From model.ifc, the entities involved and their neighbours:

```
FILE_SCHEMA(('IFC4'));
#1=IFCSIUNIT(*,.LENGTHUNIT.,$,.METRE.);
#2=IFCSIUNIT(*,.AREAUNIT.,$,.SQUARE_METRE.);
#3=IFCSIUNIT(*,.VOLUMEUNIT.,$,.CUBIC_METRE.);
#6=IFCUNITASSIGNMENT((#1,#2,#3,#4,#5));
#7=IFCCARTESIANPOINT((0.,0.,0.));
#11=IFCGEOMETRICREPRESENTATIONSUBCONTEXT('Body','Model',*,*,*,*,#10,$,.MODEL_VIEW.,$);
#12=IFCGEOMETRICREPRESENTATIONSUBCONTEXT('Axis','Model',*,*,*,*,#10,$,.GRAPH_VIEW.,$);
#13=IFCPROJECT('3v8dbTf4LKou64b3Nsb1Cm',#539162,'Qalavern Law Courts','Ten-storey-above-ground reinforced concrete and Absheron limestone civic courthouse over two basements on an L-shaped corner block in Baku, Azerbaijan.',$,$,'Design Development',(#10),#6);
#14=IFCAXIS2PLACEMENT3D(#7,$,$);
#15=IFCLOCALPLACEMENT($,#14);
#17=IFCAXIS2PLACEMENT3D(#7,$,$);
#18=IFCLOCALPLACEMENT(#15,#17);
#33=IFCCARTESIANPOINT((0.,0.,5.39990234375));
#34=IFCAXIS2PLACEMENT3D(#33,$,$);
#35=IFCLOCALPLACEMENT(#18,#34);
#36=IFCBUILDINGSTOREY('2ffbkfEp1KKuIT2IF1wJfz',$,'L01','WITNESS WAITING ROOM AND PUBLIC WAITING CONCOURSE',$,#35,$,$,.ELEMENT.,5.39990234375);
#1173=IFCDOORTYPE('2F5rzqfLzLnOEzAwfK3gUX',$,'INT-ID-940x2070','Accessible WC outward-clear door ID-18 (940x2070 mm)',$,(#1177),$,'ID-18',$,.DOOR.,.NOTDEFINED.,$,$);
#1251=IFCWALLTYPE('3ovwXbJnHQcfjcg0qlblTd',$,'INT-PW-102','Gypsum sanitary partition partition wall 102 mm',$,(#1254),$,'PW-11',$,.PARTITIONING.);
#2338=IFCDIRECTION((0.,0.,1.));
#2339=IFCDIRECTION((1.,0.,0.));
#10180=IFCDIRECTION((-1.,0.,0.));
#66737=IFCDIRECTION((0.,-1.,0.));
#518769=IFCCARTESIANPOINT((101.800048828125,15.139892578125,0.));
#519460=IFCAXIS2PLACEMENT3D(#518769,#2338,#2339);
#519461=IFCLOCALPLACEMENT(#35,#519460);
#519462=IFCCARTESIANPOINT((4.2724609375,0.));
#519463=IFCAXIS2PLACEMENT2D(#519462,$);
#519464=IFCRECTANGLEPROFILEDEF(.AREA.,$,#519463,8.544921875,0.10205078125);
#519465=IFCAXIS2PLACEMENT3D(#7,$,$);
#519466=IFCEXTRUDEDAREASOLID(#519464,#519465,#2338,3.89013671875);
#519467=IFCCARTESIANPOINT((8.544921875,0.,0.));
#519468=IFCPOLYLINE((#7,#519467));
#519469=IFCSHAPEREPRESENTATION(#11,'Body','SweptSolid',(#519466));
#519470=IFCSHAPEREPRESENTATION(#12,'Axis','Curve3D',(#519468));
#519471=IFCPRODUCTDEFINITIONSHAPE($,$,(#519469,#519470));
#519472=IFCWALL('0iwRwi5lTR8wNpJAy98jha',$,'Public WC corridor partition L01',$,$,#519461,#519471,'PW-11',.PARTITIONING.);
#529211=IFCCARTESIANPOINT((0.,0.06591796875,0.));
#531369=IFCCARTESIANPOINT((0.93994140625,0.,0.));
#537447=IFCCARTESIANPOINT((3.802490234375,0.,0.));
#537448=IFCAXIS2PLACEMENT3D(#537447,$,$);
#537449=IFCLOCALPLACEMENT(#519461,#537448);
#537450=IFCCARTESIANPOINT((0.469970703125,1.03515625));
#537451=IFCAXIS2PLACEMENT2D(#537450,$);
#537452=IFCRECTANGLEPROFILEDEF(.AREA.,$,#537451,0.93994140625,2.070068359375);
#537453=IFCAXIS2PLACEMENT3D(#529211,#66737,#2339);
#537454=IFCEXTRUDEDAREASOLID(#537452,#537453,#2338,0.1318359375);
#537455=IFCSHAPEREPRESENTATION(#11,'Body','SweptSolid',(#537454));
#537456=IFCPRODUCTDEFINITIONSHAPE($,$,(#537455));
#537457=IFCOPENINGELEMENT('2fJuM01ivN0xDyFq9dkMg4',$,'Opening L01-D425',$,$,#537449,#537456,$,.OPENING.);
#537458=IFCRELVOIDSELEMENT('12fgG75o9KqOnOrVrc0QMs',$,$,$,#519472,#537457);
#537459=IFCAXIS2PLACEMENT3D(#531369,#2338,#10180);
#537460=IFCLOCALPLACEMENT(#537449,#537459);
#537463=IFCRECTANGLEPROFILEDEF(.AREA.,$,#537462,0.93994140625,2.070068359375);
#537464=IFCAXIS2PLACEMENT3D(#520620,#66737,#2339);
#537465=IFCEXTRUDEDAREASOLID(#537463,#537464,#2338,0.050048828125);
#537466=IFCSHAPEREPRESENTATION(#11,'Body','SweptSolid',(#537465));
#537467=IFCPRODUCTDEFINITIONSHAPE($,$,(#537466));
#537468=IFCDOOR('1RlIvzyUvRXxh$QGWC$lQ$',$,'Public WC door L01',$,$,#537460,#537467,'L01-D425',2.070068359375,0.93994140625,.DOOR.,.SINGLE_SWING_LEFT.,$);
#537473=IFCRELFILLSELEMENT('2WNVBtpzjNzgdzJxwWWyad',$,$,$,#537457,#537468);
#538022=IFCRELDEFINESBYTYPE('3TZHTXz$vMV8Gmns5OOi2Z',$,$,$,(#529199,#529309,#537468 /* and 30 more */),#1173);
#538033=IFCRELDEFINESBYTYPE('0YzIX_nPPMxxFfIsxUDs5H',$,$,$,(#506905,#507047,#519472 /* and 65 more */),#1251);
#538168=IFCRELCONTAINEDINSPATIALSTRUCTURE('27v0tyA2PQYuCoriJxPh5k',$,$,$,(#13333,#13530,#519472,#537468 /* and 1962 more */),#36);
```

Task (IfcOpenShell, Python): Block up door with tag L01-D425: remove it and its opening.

```python
import ifcopenshell
import ifcopenshell.api.feature
import ifcopenshell.api.root
import ifcopenshell.geom
import ifcopenshell.util.shape

model = ifcopenshell.open("model.ifc")
settings = ifcopenshell.geom.settings()


def volume(element):
    """Net volume in cubic metres, openings subtracted."""
    shape = ifcopenshell.geom.create_shape(settings, element)
    return ifcopenshell.util.shape.get_volume(shape.geometry)


door = model.by_guid("1RlIvzyUvRXxh$QGWC$lQ$")
opening = door.FillsVoids[0].RelatingOpeningElement
wall = opening.VoidsElements[0].RelatingBuildingElement
before = volume(wall)

ifcopenshell.api.root.remove_product(model, product=door)
ifcopenshell.api.feature.remove_feature(model, feature=opening)

after = volume(wall)

print(f"wall volume {before:.3f} -> {after:.3f} m3")

model.write("model-out.ifc")
```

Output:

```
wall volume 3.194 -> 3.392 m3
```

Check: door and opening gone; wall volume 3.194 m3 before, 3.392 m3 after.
